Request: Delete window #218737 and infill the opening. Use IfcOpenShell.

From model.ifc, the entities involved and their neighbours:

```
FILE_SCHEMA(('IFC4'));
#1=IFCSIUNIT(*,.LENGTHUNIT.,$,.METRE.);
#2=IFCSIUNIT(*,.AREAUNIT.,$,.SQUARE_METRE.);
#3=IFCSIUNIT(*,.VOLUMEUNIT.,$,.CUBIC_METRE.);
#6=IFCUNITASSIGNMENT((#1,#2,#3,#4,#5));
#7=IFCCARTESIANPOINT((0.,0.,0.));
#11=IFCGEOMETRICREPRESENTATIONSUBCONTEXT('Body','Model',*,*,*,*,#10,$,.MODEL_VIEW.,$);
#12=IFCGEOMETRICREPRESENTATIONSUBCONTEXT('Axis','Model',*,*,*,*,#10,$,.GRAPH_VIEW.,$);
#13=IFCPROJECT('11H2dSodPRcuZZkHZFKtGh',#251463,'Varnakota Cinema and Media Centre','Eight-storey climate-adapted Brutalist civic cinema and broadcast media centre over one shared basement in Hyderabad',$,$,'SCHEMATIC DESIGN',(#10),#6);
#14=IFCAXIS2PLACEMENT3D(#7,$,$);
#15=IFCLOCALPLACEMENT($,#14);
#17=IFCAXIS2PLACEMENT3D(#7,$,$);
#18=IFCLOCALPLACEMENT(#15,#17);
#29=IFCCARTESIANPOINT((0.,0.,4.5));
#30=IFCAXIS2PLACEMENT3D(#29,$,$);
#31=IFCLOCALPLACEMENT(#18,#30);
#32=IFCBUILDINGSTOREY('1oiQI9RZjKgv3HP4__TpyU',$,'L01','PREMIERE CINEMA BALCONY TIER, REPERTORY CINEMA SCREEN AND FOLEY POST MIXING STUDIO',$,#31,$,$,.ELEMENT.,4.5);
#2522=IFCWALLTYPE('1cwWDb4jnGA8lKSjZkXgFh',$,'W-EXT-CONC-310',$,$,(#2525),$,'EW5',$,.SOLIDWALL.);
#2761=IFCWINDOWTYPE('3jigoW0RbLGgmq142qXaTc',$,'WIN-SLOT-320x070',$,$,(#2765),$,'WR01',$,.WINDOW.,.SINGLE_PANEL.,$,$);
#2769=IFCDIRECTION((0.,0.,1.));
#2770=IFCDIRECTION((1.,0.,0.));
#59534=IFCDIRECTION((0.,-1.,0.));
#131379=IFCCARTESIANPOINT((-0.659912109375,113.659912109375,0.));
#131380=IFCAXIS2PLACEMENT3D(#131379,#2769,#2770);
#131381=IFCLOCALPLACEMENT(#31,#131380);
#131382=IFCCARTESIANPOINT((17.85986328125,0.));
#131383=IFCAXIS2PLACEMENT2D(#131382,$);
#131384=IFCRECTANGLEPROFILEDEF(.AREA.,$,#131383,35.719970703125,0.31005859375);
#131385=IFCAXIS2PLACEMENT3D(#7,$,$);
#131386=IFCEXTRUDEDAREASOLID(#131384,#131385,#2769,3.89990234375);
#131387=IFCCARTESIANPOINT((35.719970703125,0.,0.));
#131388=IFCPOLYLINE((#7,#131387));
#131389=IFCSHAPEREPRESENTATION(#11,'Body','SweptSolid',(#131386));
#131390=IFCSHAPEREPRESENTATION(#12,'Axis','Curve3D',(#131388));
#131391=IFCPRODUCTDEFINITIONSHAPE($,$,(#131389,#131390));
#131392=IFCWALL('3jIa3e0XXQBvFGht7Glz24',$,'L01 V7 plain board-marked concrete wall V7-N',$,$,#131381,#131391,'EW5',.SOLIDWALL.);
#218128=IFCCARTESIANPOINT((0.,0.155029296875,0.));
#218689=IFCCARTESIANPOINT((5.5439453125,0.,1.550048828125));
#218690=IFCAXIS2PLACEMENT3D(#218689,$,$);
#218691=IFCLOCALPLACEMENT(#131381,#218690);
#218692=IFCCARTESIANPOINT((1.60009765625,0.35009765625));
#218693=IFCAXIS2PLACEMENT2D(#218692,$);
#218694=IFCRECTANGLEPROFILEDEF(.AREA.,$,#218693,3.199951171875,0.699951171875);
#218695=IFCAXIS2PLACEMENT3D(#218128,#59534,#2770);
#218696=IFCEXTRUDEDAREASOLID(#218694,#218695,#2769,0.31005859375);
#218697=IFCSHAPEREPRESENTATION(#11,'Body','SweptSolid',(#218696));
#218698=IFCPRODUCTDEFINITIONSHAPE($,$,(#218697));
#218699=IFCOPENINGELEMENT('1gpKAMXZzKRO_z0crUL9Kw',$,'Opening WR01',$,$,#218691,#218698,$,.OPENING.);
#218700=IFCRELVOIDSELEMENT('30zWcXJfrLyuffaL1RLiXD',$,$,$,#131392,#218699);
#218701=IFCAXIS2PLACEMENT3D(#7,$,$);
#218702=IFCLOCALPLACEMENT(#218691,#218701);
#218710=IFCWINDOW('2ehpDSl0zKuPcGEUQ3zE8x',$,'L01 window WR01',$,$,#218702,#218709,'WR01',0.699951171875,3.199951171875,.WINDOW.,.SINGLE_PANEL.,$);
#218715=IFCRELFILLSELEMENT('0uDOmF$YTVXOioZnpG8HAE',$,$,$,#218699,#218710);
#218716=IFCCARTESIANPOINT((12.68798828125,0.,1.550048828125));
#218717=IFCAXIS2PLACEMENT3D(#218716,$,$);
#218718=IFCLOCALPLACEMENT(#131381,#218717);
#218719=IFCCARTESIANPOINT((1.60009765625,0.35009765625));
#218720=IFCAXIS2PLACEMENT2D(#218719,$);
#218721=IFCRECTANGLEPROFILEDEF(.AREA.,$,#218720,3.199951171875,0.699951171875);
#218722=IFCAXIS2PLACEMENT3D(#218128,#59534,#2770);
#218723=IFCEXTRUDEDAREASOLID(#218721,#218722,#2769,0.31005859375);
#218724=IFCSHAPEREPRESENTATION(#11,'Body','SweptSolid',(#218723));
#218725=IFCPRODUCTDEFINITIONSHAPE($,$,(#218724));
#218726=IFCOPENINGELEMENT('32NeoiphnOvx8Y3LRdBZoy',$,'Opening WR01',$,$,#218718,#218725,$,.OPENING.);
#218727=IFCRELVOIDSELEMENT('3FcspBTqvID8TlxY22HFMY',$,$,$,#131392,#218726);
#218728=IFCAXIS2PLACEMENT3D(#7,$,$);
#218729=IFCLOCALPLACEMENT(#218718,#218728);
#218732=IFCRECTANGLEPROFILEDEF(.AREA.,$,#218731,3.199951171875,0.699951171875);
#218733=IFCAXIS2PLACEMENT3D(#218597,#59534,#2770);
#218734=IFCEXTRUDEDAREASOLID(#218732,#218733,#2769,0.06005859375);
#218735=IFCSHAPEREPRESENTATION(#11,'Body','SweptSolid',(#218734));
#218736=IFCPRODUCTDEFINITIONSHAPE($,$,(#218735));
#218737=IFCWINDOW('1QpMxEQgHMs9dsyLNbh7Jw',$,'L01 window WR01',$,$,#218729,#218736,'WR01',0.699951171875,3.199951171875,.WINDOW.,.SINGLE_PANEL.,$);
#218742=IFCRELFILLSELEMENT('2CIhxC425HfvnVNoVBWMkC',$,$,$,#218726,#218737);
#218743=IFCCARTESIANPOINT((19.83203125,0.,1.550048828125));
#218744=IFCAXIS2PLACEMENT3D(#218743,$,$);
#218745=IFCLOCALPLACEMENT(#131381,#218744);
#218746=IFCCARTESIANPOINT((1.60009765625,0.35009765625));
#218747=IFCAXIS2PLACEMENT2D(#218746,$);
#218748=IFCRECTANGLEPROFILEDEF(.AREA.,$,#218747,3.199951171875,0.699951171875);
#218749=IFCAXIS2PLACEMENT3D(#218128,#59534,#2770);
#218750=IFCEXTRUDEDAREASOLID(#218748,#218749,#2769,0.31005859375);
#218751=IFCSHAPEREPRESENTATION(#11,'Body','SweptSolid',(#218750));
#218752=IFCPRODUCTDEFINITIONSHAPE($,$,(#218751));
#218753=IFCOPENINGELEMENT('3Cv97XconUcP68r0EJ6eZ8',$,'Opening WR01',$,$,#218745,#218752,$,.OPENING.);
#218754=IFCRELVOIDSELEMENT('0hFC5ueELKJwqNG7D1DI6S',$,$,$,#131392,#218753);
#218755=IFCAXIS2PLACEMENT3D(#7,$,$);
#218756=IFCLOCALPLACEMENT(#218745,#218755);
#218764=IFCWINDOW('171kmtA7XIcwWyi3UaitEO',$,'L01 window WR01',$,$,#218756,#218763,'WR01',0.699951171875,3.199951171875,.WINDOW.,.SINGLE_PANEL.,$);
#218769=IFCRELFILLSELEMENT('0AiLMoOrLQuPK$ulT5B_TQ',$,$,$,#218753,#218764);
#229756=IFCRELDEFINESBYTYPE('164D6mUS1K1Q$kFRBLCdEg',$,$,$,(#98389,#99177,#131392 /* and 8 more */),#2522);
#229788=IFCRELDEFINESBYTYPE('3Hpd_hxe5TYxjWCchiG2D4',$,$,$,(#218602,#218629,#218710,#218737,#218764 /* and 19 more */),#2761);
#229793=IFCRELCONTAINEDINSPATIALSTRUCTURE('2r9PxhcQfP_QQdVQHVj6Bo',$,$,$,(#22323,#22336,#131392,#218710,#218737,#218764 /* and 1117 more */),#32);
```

```python
import ifcopenshell
import ifcopenshell.api.feature
import ifcopenshell.api.root
import ifcopenshell.geom
import ifcopenshell.util.shape

model = ifcopenshell.open("model.ifc")
settings = ifcopenshell.geom.settings()


def volume(element):
    """Net volume in cubic metres, openings subtracted."""
    shape = ifcopenshell.geom.create_shape(settings, element)
    return ifcopenshell.util.shape.get_volume(shape.geometry)


window = model.by_guid("1QpMxEQgHMs9dsyLNbh7Jw")
opening = window.FillsVoids[0].RelatingOpeningElement
wall = opening.VoidsElements[0].RelatingBuildingElement
before = volume(wall)

ifcopenshell.api.root.remove_product(model, product=window)
ifcopenshell.api.feature.remove_feature(model, feature=opening)

after = volume(wall)

print(f"wall volume {before:.3f} -> {after:.3f} m3")

model.write("model_v2.ifc")
```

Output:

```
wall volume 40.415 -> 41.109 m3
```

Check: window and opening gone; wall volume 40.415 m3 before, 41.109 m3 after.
